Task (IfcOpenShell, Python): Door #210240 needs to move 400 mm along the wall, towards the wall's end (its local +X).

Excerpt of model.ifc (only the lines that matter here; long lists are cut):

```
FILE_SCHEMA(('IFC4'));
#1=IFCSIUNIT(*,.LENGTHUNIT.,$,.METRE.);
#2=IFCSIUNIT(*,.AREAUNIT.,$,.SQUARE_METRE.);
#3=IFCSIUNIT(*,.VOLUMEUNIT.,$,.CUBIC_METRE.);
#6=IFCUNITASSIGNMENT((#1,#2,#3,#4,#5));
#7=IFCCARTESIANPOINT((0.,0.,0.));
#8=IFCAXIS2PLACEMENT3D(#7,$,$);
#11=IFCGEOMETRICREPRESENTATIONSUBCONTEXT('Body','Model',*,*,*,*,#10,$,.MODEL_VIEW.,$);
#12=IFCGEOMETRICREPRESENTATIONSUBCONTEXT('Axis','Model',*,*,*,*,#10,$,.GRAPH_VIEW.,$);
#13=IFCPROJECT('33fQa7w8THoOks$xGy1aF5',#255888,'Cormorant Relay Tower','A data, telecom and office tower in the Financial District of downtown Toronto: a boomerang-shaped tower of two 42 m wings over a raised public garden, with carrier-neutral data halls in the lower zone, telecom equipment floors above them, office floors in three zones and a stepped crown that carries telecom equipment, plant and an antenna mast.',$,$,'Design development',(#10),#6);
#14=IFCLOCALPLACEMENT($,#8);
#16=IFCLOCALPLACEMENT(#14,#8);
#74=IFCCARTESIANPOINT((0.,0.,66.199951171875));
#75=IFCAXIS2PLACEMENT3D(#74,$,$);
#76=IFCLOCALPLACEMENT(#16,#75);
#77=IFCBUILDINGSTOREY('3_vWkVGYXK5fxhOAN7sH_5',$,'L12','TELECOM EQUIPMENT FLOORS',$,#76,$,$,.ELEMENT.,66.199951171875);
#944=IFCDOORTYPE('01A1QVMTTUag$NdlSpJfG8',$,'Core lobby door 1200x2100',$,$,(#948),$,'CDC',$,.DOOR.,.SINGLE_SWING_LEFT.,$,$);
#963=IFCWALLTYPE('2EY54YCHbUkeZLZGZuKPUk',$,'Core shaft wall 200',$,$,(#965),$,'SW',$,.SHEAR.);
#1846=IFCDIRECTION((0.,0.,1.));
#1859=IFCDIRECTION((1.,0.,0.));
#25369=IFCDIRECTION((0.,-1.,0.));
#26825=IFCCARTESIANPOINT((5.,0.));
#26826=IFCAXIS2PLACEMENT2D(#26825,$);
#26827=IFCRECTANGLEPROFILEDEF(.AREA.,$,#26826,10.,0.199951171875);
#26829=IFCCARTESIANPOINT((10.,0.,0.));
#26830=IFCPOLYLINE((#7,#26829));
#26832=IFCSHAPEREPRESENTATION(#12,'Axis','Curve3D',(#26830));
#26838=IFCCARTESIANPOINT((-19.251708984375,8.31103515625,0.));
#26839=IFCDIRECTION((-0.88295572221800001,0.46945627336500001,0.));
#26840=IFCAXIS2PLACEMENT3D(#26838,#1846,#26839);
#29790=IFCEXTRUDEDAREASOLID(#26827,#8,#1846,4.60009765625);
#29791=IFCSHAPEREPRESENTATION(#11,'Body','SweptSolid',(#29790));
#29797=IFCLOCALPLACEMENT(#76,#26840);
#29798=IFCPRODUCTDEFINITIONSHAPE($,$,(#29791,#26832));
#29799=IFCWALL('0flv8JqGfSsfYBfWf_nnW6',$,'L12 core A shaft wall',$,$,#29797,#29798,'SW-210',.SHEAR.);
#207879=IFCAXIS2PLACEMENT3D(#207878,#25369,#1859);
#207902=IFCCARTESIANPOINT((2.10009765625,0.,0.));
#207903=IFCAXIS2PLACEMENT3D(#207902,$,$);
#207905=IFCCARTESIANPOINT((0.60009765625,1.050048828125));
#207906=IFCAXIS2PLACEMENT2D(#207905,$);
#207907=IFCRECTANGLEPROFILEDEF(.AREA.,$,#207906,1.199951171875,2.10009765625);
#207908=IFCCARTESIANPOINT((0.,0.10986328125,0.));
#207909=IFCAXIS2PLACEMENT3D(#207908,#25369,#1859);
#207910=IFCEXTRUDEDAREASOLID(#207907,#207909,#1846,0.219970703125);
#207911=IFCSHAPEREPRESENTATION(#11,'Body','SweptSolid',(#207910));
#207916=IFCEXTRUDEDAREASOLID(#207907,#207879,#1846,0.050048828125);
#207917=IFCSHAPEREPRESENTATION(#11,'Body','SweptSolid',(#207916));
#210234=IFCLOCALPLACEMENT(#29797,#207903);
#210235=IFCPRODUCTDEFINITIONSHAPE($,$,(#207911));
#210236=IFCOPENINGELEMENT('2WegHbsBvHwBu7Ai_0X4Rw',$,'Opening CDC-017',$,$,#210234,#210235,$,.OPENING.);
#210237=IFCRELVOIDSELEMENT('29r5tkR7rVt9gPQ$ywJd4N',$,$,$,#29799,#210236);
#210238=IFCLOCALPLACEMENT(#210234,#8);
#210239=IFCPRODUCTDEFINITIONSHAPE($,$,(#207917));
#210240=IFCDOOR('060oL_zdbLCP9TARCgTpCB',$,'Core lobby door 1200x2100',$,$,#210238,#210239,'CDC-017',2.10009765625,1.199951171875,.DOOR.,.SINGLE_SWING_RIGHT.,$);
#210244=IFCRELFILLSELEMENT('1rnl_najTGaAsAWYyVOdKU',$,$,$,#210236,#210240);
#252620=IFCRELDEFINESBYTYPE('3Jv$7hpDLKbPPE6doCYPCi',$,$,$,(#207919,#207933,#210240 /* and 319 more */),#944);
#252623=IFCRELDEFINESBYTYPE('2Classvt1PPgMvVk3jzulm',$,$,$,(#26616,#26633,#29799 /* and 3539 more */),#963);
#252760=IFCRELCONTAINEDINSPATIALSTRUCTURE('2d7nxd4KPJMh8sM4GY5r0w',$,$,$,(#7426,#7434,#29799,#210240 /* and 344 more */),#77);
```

```python
import ifcopenshell
import ifcopenshell.api.geometry
import ifcopenshell.util.placement
import ifcopenshell.util.unit

model = ifcopenshell.open("model.ifc")
unit_scale = ifcopenshell.util.unit.calculate_unit_scale(model)

door = model.by_guid("060oL_zdbLCP9TARCgTpCB")
opening = door.FillsVoids[0].RelatingOpeningElement
wall = opening.VoidsElements[0].RelatingBuildingElement

wall_matrix = ifcopenshell.util.placement.get_local_placement(wall.ObjectPlacement)
shift = wall_matrix[:3, 0] * 0.4 / unit_scale
before = ifcopenshell.util.placement.get_local_placement(door.ObjectPlacement)[:3, 3].copy()

# The door is placed relative to its opening, so it follows when the opening moves.
matrix = ifcopenshell.util.placement.get_local_placement(opening.ObjectPlacement)
matrix[:3, 3] += shift
ifcopenshell.api.geometry.edit_object_placement(
    model, product=opening, matrix=matrix, is_si=False, should_transform_children=True
)

after = ifcopenshell.util.placement.get_local_placement(door.ObjectPlacement)[:3, 3]
print("door moved by", (after - before).round(3) + 0.0)

model.write("model_rev.ifc")
```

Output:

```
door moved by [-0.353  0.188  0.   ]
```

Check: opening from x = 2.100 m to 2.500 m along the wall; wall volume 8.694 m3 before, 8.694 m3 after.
